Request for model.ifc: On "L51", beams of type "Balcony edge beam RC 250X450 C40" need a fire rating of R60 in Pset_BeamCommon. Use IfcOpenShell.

First a look at what the model holds.

```python
import ifcopenshell
import ifcopenshell.util.element

model = ifcopenshell.open("model.ifc")
print(model.schema)
storey = next(s for s in model.by_type("IfcBuildingStorey") if s.Name == "L51")
beams = [e for e in ifcopenshell.util.element.get_decomposition(storey) if e.is_a("IfcBeam")]
seen = {}
for e in beams:
    element_type = ifcopenshell.util.element.get_type(e)
    key = (element_type.Name if element_type != e and element_type else None, ifcopenshell.util.element.get_pset(e, "Pset_BeamCommon", "FireRating"))
    seen[key] = seen.get(key, 0) + 1
for (name, value), count in sorted(seen.items(), key=str):
    print(count, "x", name, "|", value)
```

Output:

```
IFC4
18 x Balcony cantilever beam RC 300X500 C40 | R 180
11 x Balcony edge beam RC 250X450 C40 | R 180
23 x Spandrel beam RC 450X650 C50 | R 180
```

```python
import ifcopenshell
import ifcopenshell.api.pset
import ifcopenshell.util.element

model = ifcopenshell.open("model.ifc")

storey = next(s for s in model.by_type("IfcBuildingStorey") if s.Name == "L51")
beams = [e for e in ifcopenshell.util.element.get_decomposition(storey) if e.is_a("IfcBeam")]

count = 0
for e in beams:
    element_type = ifcopenshell.util.element.get_type(e)
    if element_type in (None, e) or element_type.Name != "Balcony edge beam RC 250X450 C40":
        continue
    found = ifcopenshell.util.element.get_pset(e, "Pset_BeamCommon", should_inherit=False)
    if found:
        pset = model.by_id(found["id"])
        if len(ifcopenshell.util.element.get_elements_by_pset(pset)) > 1:
            pset = ifcopenshell.api.pset.unshare_pset(model, products=[e], pset=pset)[0]
    else:
        pset = ifcopenshell.api.pset.add_pset(model, product=e, name="Pset_BeamCommon")
    ifcopenshell.api.pset.edit_pset(model, pset=pset, properties={"FireRating": "R60"})
    count += 1

print(count, "beams updated")

model.write("model_v2.ifc")
```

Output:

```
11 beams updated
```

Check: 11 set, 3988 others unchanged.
